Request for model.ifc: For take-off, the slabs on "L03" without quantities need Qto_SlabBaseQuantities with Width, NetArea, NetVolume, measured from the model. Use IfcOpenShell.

First a look at what the model holds.

```python
import ifcopenshell
import ifcopenshell.util.element
import ifcopenshell.util.unit

model = ifcopenshell.open("model.ifc")
print(model.schema)
for unit_type in ("LENGTHUNIT", "AREAUNIT", "VOLUMEUNIT"):
    print(unit_type, ifcopenshell.util.unit.calculate_unit_scale(model, unit_type))
storey = next(s for s in model.by_type("IfcBuildingStorey") if s.Name == "L03")
slabs = [e for e in ifcopenshell.util.element.get_decomposition(storey) if e.is_a("IfcSlab")]
for e in sorted(slabs, key=lambda e: e.id()):
    print(e.id(), e.is_a(), e.Name, list(ifcopenshell.util.element.get_psets(e, qtos_only=True)), sep=" | ")
```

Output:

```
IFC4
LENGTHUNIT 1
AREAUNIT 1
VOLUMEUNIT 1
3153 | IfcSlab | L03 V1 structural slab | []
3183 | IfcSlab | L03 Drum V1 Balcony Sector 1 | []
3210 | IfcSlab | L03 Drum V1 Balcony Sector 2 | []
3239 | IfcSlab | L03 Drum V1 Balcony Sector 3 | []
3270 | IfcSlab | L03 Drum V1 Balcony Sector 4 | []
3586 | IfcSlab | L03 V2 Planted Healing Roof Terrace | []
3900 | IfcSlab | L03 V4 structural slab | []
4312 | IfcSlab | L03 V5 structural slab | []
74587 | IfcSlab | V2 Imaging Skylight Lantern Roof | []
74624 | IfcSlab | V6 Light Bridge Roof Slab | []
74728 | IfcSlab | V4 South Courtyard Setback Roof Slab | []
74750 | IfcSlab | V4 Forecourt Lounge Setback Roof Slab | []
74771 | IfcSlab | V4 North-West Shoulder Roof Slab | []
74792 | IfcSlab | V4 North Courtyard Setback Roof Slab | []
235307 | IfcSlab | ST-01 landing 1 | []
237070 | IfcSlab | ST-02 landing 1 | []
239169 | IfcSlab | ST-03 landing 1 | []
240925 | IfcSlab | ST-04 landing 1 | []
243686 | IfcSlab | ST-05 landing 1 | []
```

```python
import ifcopenshell
import ifcopenshell.api.pset
import ifcopenshell.geom
import ifcopenshell.util.element
import ifcopenshell.util.shape
import ifcopenshell.util.unit

model = ifcopenshell.open("model.ifc")
unit_scale = ifcopenshell.util.unit.calculate_unit_scale(model)
area_scale = ifcopenshell.util.unit.calculate_unit_scale(model, "AREAUNIT")
volume_scale = ifcopenshell.util.unit.calculate_unit_scale(model, "VOLUMEUNIT")
settings = ifcopenshell.geom.settings()

storey = next(s for s in model.by_type("IfcBuildingStorey") if s.Name == "L03")
slabs = [e for e in ifcopenshell.util.element.get_decomposition(storey) if e.is_a("IfcSlab")]

for e in sorted(slabs, key=lambda e: e.id()):
    if ifcopenshell.util.element.get_psets(e, qtos_only=True, should_inherit=False):
        continue
    # Geometry comes back in metres, in the element's own axes.
    shape = ifcopenshell.geom.create_shape(settings, e)
    values = {
        "Width": ifcopenshell.util.shape.get_z(shape.geometry) / unit_scale,
        "NetArea": ifcopenshell.util.shape.get_footprint_area(shape.geometry) / area_scale,
        "NetVolume": ifcopenshell.util.shape.get_volume(shape.geometry) / volume_scale,
    }
    qto = ifcopenshell.api.pset.add_qto(model, product=e, name="Qto_SlabBaseQuantities")
    ifcopenshell.api.pset.edit_qto(model, qto=qto, properties=values)
    print(e.id(), {k: round(v, 3) for k, v in values.items()})

model.write("model_edited.ifc")
```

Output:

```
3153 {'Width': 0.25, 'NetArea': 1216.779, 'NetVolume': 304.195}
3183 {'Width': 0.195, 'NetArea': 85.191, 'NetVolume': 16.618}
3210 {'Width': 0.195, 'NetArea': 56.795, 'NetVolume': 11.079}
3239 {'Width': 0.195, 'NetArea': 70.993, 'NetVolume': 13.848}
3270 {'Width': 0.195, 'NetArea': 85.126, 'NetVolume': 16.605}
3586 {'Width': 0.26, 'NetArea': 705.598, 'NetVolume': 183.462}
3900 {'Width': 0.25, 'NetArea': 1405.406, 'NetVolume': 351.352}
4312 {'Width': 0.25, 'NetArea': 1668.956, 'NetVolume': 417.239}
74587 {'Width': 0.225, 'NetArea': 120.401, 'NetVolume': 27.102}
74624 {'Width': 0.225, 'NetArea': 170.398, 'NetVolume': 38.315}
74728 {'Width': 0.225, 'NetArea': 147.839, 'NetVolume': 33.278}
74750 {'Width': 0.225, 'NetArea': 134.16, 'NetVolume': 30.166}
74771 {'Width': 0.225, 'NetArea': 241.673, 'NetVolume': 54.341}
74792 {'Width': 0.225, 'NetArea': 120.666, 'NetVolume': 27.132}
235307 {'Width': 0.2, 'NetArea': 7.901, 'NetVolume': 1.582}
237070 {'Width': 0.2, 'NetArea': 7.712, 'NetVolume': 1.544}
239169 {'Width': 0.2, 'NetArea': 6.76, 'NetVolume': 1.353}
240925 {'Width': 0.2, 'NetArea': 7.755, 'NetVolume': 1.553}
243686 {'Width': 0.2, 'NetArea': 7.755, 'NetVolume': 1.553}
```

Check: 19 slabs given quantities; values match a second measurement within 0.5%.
